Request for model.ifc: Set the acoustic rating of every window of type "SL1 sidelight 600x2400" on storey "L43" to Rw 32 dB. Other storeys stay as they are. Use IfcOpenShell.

First a look at what the model holds.

```python
import ifcopenshell
import ifcopenshell.util.element

model = ifcopenshell.open("model.ifc")
print(model.schema)
storey = next(s for s in model.by_type("IfcBuildingStorey") if s.Name == "L43")
windows = [e for e in ifcopenshell.util.element.get_decomposition(storey) if e.is_a("IfcWindow")]
seen = {}
for e in windows:
    element_type = ifcopenshell.util.element.get_type(e)
    key = (element_type.Name if element_type != e and element_type else None, ifcopenshell.util.element.get_pset(e, "Pset_WindowCommon", "AcousticRating"))
    seen[key] = seen.get(key, 0) + 1
for (name, value), count in sorted(seen.items(), key=str):
    print(count, "x", name, "|", value)
```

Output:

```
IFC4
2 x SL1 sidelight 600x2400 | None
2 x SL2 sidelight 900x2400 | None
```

```python
import ifcopenshell
import ifcopenshell.api.pset
import ifcopenshell.util.element

model = ifcopenshell.open("model.ifc")

storey = next(s for s in model.by_type("IfcBuildingStorey") if s.Name == "L43")
windows = [e for e in ifcopenshell.util.element.get_decomposition(storey) if e.is_a("IfcWindow")]

count = 0
for e in windows:
    element_type = ifcopenshell.util.element.get_type(e)
    if element_type in (None, e) or element_type.Name != "SL1 sidelight 600x2400":
        continue
    found = ifcopenshell.util.element.get_pset(e, "Pset_WindowCommon", should_inherit=False)
    if found:
        pset = model.by_id(found["id"])
        if len(ifcopenshell.util.element.get_elements_by_pset(pset)) > 1:
            pset = ifcopenshell.api.pset.unshare_pset(model, products=[e], pset=pset)[0]
    else:
        pset = ifcopenshell.api.pset.add_pset(model, product=e, name="Pset_WindowCommon")
    ifcopenshell.api.pset.edit_pset(model, pset=pset, properties={"AcousticRating": "Rw 32 dB"})
    count += 1

print(count, "windows updated")

model.write("model_v2.ifc")
```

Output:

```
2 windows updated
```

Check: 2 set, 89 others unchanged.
